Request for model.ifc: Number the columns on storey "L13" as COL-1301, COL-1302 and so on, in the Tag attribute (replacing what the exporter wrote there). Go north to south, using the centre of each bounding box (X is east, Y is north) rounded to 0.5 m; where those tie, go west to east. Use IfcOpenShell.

First a look at what the model holds.

```python
import ifcopenshell
import ifcopenshell.util.element
import ifcopenshell.util.placement

model = ifcopenshell.open("model.ifc")
print(model.schema)
storey = next(s for s in model.by_type("IfcBuildingStorey") if s.Name == "L13")
columns = [e for e in ifcopenshell.util.element.get_decomposition(storey) if e.is_a("IfcColumn")]
for e in sorted(columns, key=lambda e: e.id()):
    origin = ifcopenshell.util.placement.get_local_placement(e.ObjectPlacement)[:3, 3]
    print(e.id(), e.Tag, e.Name, origin.round(2) + 0.0, sep=" | ")
```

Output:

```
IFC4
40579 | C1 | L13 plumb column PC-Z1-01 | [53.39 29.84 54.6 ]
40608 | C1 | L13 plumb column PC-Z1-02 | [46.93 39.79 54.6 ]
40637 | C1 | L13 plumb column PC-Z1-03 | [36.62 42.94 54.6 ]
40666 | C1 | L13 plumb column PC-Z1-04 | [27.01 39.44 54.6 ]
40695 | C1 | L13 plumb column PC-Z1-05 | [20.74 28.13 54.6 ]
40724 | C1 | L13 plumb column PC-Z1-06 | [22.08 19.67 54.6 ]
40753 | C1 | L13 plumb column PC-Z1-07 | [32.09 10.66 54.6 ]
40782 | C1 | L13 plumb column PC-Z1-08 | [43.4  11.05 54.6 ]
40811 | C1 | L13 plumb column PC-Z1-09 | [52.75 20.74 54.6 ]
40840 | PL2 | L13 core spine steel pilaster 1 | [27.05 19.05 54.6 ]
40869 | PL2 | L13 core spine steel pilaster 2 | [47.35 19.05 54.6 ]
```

```python
import ifcopenshell
import ifcopenshell.geom
import ifcopenshell.util.element
import ifcopenshell.util.shape

model = ifcopenshell.open("model.ifc")
settings = ifcopenshell.geom.settings()
settings.set("use-world-coords", True)


def centre(element):
    shape = ifcopenshell.geom.create_shape(settings, element)
    return ifcopenshell.util.shape.get_bbox_centroid(shape.geometry)


storey = next(s for s in model.by_type("IfcBuildingStorey") if s.Name == "L13")
columns = [e for e in ifcopenshell.util.element.get_decomposition(storey) if e.is_a("IfcColumn")]

# Insertion points can sit at a corner or the storey origin, so sort by the geometry (in metres).
centres = {e: centre(e) for e in columns}
columns.sort(key=lambda e: (-round(centres[e][1] / 0.5), centres[e][0]))

for i, e in enumerate(columns, start=1):
    number = f"COL-13{i:02d}"
    e.Tag = number
    print(e.id(), number)

model.write("model-out.ifc")
```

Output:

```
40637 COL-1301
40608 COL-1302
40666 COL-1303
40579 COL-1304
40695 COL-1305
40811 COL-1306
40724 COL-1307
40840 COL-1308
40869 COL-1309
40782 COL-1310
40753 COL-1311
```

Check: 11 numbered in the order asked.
